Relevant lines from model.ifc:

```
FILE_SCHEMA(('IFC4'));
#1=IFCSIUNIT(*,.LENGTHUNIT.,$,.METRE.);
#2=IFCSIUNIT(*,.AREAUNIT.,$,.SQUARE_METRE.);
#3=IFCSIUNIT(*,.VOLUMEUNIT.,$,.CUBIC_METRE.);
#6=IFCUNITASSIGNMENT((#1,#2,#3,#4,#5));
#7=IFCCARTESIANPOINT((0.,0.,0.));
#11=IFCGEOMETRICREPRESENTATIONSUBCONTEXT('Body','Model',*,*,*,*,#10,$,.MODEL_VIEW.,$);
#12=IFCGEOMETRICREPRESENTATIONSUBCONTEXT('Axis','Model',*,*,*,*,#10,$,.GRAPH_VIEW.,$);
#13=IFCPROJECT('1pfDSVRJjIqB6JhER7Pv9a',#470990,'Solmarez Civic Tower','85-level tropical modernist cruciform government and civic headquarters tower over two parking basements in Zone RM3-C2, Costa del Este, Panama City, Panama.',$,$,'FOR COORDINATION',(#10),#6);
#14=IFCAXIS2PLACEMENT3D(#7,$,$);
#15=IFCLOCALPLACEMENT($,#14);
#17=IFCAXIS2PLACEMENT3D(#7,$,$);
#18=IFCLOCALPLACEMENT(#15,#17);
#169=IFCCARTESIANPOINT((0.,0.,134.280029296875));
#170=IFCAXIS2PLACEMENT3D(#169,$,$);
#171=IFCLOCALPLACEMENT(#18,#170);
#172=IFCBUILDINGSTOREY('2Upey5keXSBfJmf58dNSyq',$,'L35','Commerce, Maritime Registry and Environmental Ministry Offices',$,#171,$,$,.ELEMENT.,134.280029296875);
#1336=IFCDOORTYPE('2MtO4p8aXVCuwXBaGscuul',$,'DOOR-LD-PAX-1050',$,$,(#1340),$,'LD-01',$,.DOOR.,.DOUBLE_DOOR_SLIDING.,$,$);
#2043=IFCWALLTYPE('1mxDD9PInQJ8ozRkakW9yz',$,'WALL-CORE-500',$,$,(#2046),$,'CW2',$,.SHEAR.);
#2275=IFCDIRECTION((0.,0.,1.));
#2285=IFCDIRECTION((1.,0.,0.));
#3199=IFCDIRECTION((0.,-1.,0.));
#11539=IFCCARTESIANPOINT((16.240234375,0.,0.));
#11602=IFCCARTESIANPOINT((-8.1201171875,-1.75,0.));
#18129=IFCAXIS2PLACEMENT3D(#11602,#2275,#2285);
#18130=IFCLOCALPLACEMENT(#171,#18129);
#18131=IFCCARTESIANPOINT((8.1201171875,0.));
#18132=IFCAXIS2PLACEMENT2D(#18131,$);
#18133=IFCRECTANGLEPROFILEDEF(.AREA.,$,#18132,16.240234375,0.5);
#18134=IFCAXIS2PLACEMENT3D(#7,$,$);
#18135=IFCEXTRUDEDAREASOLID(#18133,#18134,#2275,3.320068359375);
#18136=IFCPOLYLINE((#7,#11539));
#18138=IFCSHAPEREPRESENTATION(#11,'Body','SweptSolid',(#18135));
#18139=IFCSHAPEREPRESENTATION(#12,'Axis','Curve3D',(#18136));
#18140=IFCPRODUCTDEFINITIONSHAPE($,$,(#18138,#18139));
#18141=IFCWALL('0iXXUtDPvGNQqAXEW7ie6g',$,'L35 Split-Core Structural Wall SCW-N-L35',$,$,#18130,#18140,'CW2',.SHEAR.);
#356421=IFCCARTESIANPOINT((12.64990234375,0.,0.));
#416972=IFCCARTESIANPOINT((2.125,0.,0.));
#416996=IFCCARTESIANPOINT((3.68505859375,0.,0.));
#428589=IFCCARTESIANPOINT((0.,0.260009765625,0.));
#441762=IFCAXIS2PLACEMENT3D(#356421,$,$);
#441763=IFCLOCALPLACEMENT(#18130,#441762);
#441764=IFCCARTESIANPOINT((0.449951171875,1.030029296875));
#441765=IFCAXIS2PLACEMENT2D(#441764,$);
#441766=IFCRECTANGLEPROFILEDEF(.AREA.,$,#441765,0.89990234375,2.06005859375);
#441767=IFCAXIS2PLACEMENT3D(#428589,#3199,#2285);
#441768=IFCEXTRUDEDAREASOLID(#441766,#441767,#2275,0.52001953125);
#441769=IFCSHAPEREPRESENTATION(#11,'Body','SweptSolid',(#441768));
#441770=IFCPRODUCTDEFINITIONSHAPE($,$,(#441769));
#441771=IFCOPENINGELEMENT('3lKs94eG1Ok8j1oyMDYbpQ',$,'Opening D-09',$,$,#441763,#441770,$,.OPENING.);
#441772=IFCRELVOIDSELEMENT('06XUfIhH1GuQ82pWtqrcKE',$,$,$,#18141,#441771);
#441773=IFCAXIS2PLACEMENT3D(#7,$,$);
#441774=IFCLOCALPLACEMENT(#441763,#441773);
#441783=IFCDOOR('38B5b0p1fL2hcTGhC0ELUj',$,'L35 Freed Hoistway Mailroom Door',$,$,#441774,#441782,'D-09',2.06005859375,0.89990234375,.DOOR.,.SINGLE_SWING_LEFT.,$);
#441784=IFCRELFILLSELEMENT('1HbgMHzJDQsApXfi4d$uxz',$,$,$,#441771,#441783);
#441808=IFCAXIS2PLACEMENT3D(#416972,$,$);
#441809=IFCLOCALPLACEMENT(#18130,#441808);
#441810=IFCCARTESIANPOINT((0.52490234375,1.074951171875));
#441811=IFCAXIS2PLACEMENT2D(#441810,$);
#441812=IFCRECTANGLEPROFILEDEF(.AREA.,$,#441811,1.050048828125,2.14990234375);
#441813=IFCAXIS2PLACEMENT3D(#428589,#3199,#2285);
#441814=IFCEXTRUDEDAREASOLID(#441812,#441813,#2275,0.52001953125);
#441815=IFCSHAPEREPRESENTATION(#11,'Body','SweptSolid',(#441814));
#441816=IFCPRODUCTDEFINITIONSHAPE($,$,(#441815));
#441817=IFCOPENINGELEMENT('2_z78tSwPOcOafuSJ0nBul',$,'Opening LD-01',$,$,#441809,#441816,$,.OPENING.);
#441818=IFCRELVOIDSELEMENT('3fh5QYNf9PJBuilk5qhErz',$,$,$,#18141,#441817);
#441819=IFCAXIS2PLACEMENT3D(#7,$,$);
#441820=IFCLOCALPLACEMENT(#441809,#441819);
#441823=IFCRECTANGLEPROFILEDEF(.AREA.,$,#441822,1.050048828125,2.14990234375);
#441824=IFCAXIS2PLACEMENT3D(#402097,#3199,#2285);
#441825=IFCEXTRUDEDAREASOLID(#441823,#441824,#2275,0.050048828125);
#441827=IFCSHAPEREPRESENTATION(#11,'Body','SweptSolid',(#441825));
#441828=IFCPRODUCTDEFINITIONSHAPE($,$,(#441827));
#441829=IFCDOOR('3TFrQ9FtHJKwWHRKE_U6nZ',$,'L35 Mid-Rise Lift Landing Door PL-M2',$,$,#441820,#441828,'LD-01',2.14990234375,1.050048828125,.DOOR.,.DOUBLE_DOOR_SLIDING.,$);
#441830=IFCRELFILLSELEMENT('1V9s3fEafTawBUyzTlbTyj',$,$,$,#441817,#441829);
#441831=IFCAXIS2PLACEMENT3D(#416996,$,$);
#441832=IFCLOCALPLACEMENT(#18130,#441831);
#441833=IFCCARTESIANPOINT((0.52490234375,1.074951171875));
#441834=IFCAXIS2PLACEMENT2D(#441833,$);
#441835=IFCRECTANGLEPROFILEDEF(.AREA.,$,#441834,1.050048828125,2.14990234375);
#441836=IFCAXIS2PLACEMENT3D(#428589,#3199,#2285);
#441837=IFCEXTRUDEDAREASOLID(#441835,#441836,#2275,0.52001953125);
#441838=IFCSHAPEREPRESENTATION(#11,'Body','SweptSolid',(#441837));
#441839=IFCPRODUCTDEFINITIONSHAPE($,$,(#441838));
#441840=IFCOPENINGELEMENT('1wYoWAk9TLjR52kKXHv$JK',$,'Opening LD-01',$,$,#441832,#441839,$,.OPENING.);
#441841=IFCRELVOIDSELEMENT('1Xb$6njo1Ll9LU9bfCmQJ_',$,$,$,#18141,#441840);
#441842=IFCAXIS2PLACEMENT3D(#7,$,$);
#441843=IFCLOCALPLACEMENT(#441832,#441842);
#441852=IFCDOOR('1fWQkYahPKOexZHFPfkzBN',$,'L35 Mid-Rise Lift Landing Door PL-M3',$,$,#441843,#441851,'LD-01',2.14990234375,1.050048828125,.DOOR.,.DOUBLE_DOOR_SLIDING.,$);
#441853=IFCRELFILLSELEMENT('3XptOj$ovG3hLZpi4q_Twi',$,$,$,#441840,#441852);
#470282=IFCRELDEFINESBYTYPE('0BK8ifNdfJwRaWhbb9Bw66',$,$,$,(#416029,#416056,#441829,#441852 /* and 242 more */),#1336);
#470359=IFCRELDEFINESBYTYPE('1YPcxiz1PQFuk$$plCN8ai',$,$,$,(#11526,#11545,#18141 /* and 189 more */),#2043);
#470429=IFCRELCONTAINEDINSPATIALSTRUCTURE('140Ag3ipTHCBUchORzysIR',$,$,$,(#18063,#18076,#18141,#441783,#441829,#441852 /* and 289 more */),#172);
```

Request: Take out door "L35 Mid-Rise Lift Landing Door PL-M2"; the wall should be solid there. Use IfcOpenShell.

```python
import ifcopenshell
import ifcopenshell.api.feature
import ifcopenshell.api.root
import ifcopenshell.geom
import ifcopenshell.util.shape

model = ifcopenshell.open("model.ifc")
settings = ifcopenshell.geom.settings()


def volume(element):
    """Net volume in cubic metres, openings subtracted."""
    shape = ifcopenshell.geom.create_shape(settings, element)
    return ifcopenshell.util.shape.get_volume(shape.geometry)


door = model.by_guid("3TFrQ9FtHJKwWHRKE_U6nZ")
opening = door.FillsVoids[0].RelatingOpeningElement
wall = opening.VoidsElements[0].RelatingBuildingElement
before = volume(wall)

ifcopenshell.api.root.remove_product(model, product=door)
ifcopenshell.api.feature.remove_feature(model, feature=opening)

after = volume(wall)

print(f"wall volume {before:.3f} -> {after:.3f} m3")

model.write("model_rev.ifc")
```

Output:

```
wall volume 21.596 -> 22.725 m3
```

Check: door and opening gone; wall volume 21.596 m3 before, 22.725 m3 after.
